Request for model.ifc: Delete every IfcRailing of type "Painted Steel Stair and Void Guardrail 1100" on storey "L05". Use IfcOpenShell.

First a look at what the model holds.

```python
import ifcopenshell
import ifcopenshell.util.element

model = ifcopenshell.open("model.ifc")
print(model.schema)
storey = next(s for s in model.by_type("IfcBuildingStorey") if s.Name == "L05")
railings = [e for e in ifcopenshell.util.element.get_decomposition(storey) if e.is_a("IfcRailing")]
seen = {}
for e in railings:
    element_type = ifcopenshell.util.element.get_type(e)
    name = element_type.Name if element_type not in (None, e) else None
    seen[name] = seen.get(name, 0) + 1
for name, count in sorted(seen.items(), key=str):
    print(count, "x", name)
```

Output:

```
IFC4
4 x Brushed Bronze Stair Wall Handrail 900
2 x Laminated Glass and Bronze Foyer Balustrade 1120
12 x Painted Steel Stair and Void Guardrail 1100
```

```python
import ifcopenshell
import ifcopenshell.api.root
import ifcopenshell.util.element

model = ifcopenshell.open("model.ifc")

storey = next(s for s in model.by_type("IfcBuildingStorey") if s.Name == "L05")
railings = [e for e in ifcopenshell.util.element.get_decomposition(storey) if e.is_a("IfcRailing")]
targets = [e for e in railings if (t := ifcopenshell.util.element.get_type(e)) not in (None, e) and t.Name == "Painted Steel Stair and Void Guardrail 1100"]

for e in targets:
    ifcopenshell.api.root.remove_product(model, product=e)
print(len(targets), "removed")

model.write("model_rev.ifc")
```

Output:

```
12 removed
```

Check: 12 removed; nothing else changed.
